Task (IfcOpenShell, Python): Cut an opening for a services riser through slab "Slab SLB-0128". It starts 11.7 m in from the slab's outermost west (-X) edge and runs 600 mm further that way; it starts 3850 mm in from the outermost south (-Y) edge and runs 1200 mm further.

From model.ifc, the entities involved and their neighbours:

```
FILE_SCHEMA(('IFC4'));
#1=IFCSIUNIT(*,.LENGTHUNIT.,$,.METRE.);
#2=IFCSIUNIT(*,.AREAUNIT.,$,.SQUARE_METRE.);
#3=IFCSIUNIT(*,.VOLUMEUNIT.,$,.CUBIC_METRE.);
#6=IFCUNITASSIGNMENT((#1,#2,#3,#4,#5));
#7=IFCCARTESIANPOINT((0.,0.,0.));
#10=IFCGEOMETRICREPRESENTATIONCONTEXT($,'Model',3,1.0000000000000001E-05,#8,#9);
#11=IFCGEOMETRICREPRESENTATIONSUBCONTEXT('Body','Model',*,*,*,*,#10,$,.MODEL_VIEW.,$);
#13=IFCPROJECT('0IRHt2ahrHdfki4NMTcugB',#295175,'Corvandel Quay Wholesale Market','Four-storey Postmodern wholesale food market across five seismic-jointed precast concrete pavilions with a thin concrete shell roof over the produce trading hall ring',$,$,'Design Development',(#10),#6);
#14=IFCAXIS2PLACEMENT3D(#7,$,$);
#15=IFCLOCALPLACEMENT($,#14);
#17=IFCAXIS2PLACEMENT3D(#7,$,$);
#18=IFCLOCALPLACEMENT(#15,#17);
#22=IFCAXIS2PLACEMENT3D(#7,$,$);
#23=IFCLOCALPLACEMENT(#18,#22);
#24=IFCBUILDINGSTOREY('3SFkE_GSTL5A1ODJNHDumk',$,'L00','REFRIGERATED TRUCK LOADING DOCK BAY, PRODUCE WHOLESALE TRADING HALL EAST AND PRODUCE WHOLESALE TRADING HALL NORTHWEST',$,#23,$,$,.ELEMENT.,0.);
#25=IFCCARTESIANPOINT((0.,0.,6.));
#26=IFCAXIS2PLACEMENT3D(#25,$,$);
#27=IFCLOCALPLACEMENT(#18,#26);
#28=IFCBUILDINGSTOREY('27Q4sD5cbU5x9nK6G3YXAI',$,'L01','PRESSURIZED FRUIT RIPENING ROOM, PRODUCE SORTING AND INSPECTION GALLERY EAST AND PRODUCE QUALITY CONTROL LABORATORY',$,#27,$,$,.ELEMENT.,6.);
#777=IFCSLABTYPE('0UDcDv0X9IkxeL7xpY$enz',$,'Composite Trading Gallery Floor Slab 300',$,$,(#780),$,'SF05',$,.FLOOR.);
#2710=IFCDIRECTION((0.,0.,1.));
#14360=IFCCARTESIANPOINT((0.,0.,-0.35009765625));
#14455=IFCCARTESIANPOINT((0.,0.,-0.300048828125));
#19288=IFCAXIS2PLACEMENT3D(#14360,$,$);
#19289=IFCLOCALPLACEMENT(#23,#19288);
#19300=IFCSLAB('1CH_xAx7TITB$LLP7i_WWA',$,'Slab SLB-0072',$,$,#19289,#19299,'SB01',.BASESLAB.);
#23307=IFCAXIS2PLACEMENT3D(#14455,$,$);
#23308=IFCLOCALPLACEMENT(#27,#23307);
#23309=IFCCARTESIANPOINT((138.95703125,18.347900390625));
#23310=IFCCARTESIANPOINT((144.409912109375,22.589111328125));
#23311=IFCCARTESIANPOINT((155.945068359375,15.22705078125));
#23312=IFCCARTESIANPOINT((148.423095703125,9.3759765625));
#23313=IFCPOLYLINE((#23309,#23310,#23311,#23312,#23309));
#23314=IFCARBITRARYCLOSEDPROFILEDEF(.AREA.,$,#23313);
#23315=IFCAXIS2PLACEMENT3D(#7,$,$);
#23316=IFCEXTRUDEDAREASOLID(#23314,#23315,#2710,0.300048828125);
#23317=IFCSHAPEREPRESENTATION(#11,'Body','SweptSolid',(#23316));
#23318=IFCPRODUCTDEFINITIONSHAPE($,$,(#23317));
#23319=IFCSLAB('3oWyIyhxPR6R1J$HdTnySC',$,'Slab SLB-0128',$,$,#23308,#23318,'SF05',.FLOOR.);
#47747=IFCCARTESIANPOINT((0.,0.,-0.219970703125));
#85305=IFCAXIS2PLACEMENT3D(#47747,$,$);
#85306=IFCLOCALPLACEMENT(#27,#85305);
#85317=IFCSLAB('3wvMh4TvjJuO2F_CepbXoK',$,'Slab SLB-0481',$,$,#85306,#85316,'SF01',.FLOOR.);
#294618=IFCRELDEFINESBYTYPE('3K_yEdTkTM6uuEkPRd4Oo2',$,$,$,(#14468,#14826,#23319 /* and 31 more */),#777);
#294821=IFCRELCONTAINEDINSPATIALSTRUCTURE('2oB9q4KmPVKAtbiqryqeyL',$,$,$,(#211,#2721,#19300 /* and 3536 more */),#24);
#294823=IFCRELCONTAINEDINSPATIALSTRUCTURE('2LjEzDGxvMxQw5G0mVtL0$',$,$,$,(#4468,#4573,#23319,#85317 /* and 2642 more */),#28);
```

```python
import numpy as np
import ifcopenshell
import ifcopenshell.api.feature
import ifcopenshell.api.geometry
import ifcopenshell.api.root
import ifcopenshell.geom
import ifcopenshell.util.placement
import ifcopenshell.util.representation
import ifcopenshell.util.shape
import ifcopenshell.util.unit

model = ifcopenshell.open("model.ifc")
unit_scale = ifcopenshell.util.unit.calculate_unit_scale(model)
settings = ifcopenshell.geom.settings()


def volume(element):
    """Net volume in cubic metres, openings subtracted."""
    shape = ifcopenshell.geom.create_shape(settings, element)
    return ifcopenshell.util.shape.get_volume(shape.geometry)


slab = model.by_guid("3oWyIyhxPR6R1J$HdTnySC")
before = volume(slab)

# Extent in the slab's own axes, in metres. The edges named are its -X and -Y sides.
slab_shape = ifcopenshell.geom.create_shape(settings, slab)
vertices = ifcopenshell.util.shape.get_vertices(slab_shape.geometry)
x_min, y_min, bottom = vertices.min(axis=0)
top = vertices[:, 2].max()

opening = ifcopenshell.api.root.create_entity(model, ifc_class="IfcOpeningElement", name="Services riser opening", predefined_type="OPENING")
context = ifcopenshell.util.representation.get_context(model, "Model", "Body", "MODEL_VIEW")
width, depth = 0.6, 1.2
outline = [(0.0, 0.0), (width, 0.0), (width, depth), (0.0, depth), (0.0, 0.0)]
# Overshoot both faces by 50 mm so the cut is clean.
shape = ifcopenshell.api.geometry.add_slab_representation(
    model, context=context, depth=top - bottom + 0.1, polyline=outline
)
ifcopenshell.api.geometry.assign_representation(model, product=opening, representation=shape)

matrix = ifcopenshell.util.placement.get_local_placement(slab.ObjectPlacement)
matrix[:, 3] = matrix @ np.append(np.array([x_min + 11.7, y_min + 3.85, bottom - 0.05]) / unit_scale, 1.0)
ifcopenshell.api.geometry.edit_object_placement(model, product=opening, matrix=matrix, is_si=False)
ifcopenshell.api.feature.add_feature(model, feature=opening, element=slab)

after = volume(slab)

print(f"slab volume {before:.3f} -> {after:.3f} m3")

model.write("model_rev.ifc")
```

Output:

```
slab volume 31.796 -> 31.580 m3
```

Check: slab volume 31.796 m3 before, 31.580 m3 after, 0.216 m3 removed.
